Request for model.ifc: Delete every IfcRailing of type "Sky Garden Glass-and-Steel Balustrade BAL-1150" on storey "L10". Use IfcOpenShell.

First a look at what the model holds.

```python
import ifcopenshell
import ifcopenshell.util.element

model = ifcopenshell.open("model.ifc")
print(model.schema)
storey = next(s for s in model.by_type("IfcBuildingStorey") if s.Name == "L10")
railings = [e for e in ifcopenshell.util.element.get_decomposition(storey) if e.is_a("IfcRailing")]
seen = {}
for e in railings:
    element_type = ifcopenshell.util.element.get_type(e)
    name = element_type.Name if element_type not in (None, e) else None
    seen[name] = seen.get(name, 0) + 1
for name, count in sorted(seen.items(), key=str):
    print(count, "x", name)
```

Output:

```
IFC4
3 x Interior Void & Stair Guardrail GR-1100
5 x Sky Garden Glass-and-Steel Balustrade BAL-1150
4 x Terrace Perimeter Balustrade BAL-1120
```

```python
import ifcopenshell
import ifcopenshell.api.root
import ifcopenshell.util.element

model = ifcopenshell.open("model.ifc")

storey = next(s for s in model.by_type("IfcBuildingStorey") if s.Name == "L10")
railings = [e for e in ifcopenshell.util.element.get_decomposition(storey) if e.is_a("IfcRailing")]
targets = [e for e in railings if (t := ifcopenshell.util.element.get_type(e)) not in (None, e) and t.Name == "Sky Garden Glass-and-Steel Balustrade BAL-1150"]

for e in targets:
    ifcopenshell.api.root.remove_product(model, product=e)
print(len(targets), "removed")

model.write("model-out.ifc")
```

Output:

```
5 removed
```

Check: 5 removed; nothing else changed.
